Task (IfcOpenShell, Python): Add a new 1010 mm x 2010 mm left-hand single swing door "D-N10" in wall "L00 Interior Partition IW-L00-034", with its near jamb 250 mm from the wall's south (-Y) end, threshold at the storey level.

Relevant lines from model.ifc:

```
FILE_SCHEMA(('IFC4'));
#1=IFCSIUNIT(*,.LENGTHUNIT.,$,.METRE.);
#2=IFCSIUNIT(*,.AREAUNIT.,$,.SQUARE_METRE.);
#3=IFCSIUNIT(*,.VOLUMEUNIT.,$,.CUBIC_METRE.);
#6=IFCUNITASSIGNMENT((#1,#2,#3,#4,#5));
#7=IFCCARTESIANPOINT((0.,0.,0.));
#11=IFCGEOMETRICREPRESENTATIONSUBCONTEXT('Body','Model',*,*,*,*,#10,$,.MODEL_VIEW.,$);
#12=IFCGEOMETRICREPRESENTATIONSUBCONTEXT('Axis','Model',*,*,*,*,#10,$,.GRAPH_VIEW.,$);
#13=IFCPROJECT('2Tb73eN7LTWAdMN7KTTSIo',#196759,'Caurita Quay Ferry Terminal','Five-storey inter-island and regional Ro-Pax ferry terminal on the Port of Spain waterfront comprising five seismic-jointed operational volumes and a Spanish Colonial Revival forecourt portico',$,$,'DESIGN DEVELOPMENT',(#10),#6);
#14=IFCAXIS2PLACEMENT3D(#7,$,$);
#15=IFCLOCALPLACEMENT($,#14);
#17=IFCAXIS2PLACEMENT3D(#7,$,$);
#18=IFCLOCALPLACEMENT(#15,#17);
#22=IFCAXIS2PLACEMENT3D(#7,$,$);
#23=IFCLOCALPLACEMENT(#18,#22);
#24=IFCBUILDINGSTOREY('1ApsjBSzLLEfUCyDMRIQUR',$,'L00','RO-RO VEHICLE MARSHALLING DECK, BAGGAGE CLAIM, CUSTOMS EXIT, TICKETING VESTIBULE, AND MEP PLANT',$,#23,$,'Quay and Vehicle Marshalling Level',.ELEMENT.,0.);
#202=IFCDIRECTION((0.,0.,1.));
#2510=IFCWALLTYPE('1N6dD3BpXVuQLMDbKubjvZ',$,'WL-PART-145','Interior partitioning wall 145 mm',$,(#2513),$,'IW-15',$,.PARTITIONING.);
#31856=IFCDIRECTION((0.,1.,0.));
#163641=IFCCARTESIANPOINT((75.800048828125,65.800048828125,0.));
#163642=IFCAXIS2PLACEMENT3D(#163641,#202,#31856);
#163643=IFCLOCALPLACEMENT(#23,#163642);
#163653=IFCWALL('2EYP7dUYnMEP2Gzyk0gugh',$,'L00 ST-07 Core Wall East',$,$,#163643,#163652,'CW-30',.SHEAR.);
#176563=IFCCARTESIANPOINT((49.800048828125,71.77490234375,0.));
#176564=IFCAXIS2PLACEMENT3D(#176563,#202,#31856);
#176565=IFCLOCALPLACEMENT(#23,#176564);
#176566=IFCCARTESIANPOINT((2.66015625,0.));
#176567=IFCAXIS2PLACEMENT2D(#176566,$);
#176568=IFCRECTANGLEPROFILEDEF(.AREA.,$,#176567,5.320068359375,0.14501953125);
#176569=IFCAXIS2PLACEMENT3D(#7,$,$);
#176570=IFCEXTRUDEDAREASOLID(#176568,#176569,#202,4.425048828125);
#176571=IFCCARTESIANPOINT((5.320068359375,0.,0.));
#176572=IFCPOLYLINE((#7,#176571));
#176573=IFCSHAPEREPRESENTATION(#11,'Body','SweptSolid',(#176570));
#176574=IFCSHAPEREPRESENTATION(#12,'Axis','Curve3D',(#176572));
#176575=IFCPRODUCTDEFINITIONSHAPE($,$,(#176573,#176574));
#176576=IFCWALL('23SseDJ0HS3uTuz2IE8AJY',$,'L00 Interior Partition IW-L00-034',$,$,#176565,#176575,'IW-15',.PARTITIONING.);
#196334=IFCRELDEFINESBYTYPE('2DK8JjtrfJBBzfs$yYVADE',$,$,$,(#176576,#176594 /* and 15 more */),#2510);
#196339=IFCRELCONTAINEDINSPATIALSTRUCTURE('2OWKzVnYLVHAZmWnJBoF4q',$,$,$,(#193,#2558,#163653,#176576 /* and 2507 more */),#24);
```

```python
import numpy as np
import ifcopenshell
import ifcopenshell.api.feature
import ifcopenshell.api.geometry
import ifcopenshell.api.root
import ifcopenshell.api.spatial
import ifcopenshell.geom
import ifcopenshell.util.element
import ifcopenshell.util.placement
import ifcopenshell.util.representation
import ifcopenshell.util.shape
import ifcopenshell.util.unit

model = ifcopenshell.open("model.ifc")
unit_scale = ifcopenshell.util.unit.calculate_unit_scale(model)
settings = ifcopenshell.geom.settings()


def volume(element):
    """Net volume in cubic metres, openings subtracted."""
    shape = ifcopenshell.geom.create_shape(settings, element)
    return ifcopenshell.util.shape.get_volume(shape.geometry)


wall = model.by_guid("23SseDJ0HS3uTuz2IE8AJY")
storey = ifcopenshell.util.element.get_container(wall, ifc_class="IfcBuildingStorey")
context = ifcopenshell.util.representation.get_context(model, "Model", "Body", "MODEL_VIEW")
before = volume(wall)

width, height, from_end, sill = 1.01, 2.01, 0.25, 0.0  # metres

# The wall runs along its own X axis, and the end named is its -X end.
wall_shape = ifcopenshell.geom.create_shape(settings, wall)
x, y, z = ifcopenshell.util.shape.get_vertices(wall_shape.geometry).T
start = x.min() + from_end
face, thickness = float(y.min()), float(y.max() - y.min())
wall_matrix = ifcopenshell.util.placement.get_local_placement(wall.ObjectPlacement)
level = ifcopenshell.util.placement.get_local_placement(storey.ObjectPlacement)[2, 3]


def in_wall(x, y):
    """Placement at x, y metres in the wall's axes, at sill height."""
    matrix = wall_matrix.copy()
    matrix[:, 3] = wall_matrix @ np.array([x / unit_scale, y / unit_scale, 0.0, 1.0])
    matrix[2, 3] = level + sill / unit_scale
    return matrix


# Opening: a box that overshoots both wall faces by 50 mm.
opening = ifcopenshell.api.root.create_entity(model, ifc_class="IfcOpeningElement", predefined_type="OPENING")
box = ifcopenshell.api.geometry.add_wall_representation(
    model, context=context, length=width, height=height, thickness=thickness + 0.1
)
ifcopenshell.api.geometry.assign_representation(model, product=opening, representation=box)
ifcopenshell.api.geometry.edit_object_placement(model, product=opening, matrix=in_wall(start, face - 0.05), is_si=False)
ifcopenshell.api.feature.add_feature(model, feature=opening, element=wall)

door = ifcopenshell.api.root.create_entity(model, ifc_class="IfcDoor", name="D-N10", predefined_type="DOOR")
door.OverallWidth, door.OverallHeight = width / unit_scale, height / unit_scale
door.OperationType = "SINGLE_SWING_LEFT"
body = ifcopenshell.api.geometry.add_door_representation(
    model,
    context=context,
    overall_width=door.OverallWidth,
    overall_height=door.OverallHeight,
    operation_type="SINGLE_SWING_LEFT",
    lining_properties={"LiningDepth": thickness / unit_scale, "ThresholdDepth": thickness / unit_scale},
)
ifcopenshell.api.geometry.assign_representation(model, product=door, representation=body)
ifcopenshell.api.spatial.assign_container(model, products=[door], relating_structure=storey)
ifcopenshell.api.feature.add_filling(model, opening=opening, element=door)

# The lining spans the wall, so the door starts at the wall face.
ifcopenshell.api.geometry.edit_object_placement(model, product=door, matrix=in_wall(start, face), is_si=False)

after = volume(wall)

print(f"wall volume {before:.3f} -> {after:.3f} m3")

model.write("model_edited.ifc")
```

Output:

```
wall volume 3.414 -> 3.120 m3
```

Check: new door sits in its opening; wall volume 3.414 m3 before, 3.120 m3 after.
